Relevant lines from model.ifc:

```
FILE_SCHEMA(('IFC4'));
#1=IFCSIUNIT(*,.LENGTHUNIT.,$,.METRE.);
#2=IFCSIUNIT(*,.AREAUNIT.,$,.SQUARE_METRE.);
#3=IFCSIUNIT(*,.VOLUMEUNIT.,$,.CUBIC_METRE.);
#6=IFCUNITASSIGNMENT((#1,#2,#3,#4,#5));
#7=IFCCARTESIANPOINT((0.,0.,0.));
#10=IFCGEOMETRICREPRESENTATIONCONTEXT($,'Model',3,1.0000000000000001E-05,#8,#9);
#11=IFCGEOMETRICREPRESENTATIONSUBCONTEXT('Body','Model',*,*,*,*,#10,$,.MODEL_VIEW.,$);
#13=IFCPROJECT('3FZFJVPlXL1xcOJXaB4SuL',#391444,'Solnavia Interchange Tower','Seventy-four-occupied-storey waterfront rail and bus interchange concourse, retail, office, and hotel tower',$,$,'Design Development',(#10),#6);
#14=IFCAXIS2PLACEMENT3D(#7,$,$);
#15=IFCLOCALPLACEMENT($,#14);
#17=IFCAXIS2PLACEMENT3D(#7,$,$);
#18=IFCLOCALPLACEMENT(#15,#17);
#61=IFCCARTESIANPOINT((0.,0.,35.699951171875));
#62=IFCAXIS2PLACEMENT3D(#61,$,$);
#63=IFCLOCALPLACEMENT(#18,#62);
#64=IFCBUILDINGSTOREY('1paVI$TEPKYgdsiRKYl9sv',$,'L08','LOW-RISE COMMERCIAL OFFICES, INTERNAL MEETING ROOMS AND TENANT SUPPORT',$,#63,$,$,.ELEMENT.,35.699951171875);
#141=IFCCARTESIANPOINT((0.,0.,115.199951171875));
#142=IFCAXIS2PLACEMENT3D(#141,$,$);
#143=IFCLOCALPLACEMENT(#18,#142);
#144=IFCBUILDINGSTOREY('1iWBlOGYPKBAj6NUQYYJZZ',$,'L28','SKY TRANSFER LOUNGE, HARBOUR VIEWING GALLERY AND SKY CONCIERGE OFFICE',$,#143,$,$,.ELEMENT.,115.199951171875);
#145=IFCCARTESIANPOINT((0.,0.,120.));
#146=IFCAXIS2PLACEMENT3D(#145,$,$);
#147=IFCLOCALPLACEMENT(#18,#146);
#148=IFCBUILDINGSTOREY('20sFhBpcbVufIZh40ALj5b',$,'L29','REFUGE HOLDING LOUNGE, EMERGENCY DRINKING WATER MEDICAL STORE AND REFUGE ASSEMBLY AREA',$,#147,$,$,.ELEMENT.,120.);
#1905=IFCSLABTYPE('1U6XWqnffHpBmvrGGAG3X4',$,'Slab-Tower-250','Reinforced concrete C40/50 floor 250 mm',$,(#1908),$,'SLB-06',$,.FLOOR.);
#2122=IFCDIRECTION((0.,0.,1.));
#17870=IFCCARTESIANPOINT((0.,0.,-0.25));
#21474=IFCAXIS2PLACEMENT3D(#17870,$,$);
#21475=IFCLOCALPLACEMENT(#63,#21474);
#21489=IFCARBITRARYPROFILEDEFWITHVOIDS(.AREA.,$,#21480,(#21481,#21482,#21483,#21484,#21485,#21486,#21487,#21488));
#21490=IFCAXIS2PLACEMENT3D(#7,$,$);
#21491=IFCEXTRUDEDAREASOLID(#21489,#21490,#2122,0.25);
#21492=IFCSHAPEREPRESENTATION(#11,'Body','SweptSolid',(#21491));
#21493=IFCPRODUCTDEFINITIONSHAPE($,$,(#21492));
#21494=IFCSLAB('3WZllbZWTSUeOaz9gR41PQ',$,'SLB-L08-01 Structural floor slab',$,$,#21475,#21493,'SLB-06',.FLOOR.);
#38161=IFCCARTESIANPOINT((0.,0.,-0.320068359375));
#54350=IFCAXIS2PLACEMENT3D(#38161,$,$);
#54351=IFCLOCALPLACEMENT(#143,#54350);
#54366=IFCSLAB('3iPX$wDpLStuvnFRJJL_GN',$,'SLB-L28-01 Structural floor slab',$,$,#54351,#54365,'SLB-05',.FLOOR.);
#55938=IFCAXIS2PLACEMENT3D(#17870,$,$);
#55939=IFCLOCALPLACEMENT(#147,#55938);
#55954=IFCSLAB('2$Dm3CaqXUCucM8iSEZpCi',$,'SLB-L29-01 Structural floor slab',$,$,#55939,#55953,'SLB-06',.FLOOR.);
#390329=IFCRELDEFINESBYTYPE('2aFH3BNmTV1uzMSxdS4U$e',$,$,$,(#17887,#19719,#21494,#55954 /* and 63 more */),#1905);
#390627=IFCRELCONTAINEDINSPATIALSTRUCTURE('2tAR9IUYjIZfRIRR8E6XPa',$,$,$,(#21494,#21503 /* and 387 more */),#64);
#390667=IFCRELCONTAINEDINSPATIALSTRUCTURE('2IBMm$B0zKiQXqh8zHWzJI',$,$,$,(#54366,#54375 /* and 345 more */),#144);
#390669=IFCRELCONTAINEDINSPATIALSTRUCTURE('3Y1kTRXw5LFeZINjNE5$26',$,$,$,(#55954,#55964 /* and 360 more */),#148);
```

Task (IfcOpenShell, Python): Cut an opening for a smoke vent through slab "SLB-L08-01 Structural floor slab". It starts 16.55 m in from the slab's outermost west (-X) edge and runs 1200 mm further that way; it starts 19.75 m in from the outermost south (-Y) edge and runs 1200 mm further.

```python
import numpy as np
import ifcopenshell
import ifcopenshell.api.feature
import ifcopenshell.api.geometry
import ifcopenshell.api.root
import ifcopenshell.geom
import ifcopenshell.util.placement
import ifcopenshell.util.representation
import ifcopenshell.util.shape
import ifcopenshell.util.unit

model = ifcopenshell.open("model.ifc")
unit_scale = ifcopenshell.util.unit.calculate_unit_scale(model)
settings = ifcopenshell.geom.settings()


def volume(element):
    """Net volume in cubic metres, openings subtracted."""
    shape = ifcopenshell.geom.create_shape(settings, element)
    return ifcopenshell.util.shape.get_volume(shape.geometry)


slab = model.by_guid("3WZllbZWTSUeOaz9gR41PQ")
before = volume(slab)

# Extent in the slab's own axes, in metres. The edges named are its -X and -Y sides.
slab_shape = ifcopenshell.geom.create_shape(settings, slab)
vertices = ifcopenshell.util.shape.get_vertices(slab_shape.geometry)
x_min, y_min, bottom = vertices.min(axis=0)
top = vertices[:, 2].max()

opening = ifcopenshell.api.root.create_entity(model, ifc_class="IfcOpeningElement", name="Smoke vent opening", predefined_type="OPENING")
context = ifcopenshell.util.representation.get_context(model, "Model", "Body", "MODEL_VIEW")
width, depth = 1.2, 1.2
outline = [(0.0, 0.0), (width, 0.0), (width, depth), (0.0, depth), (0.0, 0.0)]
# Overshoot both faces by 50 mm so the cut is clean.
shape = ifcopenshell.api.geometry.add_slab_representation(
    model, context=context, depth=top - bottom + 0.1, polyline=outline
)
ifcopenshell.api.geometry.assign_representation(model, product=opening, representation=shape)

matrix = ifcopenshell.util.placement.get_local_placement(slab.ObjectPlacement)
matrix[:, 3] = matrix @ np.append(np.array([x_min + 16.55, y_min + 19.75, bottom - 0.05]) / unit_scale, 1.0)
ifcopenshell.api.geometry.edit_object_placement(model, product=opening, matrix=matrix, is_si=False)
ifcopenshell.api.feature.add_feature(model, feature=opening, element=slab)

after = volume(slab)

print(f"slab volume {before:.3f} -> {after:.3f} m3")

model.write("model_edited.ifc")
```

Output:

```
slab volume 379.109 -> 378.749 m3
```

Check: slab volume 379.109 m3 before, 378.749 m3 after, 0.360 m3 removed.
